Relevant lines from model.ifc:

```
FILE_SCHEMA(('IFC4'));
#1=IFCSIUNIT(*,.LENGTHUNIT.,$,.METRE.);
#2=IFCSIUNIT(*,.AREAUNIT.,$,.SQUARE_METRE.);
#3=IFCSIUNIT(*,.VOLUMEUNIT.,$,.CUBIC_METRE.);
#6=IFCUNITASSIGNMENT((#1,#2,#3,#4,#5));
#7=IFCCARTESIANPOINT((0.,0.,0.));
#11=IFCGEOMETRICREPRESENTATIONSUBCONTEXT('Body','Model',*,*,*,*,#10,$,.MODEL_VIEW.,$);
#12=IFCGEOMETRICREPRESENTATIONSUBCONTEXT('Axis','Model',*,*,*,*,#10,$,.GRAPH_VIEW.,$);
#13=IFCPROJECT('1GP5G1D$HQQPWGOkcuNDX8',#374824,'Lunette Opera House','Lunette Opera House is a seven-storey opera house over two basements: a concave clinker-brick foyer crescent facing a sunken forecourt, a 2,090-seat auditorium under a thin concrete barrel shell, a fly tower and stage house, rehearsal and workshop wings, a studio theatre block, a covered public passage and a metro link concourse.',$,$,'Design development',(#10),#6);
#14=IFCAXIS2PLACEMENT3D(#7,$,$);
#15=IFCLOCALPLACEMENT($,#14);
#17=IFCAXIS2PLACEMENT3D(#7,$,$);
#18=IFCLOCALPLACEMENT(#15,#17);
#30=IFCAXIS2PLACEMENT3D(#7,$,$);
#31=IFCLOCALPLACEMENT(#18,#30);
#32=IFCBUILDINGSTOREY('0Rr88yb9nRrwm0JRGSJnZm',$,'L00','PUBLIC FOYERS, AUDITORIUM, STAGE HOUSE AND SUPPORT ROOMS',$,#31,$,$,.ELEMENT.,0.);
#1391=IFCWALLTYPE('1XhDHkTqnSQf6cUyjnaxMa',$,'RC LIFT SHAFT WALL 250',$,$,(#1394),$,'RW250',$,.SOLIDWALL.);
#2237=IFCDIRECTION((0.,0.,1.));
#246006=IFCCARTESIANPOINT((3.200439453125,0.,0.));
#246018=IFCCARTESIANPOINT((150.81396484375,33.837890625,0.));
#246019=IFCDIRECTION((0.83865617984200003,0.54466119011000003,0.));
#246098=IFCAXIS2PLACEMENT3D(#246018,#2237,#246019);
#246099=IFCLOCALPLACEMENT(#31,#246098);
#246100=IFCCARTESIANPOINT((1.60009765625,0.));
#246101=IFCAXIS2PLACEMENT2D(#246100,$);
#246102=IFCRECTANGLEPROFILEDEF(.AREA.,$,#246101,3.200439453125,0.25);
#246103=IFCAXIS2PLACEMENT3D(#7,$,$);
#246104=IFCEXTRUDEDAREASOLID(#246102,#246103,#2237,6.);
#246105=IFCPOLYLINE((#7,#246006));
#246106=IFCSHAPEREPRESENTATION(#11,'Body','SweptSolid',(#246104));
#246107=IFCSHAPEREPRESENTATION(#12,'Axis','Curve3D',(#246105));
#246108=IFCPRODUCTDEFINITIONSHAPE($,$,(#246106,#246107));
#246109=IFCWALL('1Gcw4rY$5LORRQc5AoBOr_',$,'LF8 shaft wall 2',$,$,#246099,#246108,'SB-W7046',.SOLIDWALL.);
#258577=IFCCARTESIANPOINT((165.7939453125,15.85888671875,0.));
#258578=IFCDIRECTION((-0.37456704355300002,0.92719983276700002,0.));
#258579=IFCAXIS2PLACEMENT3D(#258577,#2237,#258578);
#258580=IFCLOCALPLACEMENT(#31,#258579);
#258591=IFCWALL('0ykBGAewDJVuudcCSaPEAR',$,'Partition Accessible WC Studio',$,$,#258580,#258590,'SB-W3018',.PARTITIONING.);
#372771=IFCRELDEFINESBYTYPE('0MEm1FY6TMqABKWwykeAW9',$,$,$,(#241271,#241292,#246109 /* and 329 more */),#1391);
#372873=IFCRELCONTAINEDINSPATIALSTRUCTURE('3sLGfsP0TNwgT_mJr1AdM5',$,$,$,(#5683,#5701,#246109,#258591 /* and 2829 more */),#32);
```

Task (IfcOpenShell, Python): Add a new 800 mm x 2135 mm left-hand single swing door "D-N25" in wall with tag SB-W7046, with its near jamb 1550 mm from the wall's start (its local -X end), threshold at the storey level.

```python
import numpy as np
import ifcopenshell
import ifcopenshell.api.feature
import ifcopenshell.api.geometry
import ifcopenshell.api.root
import ifcopenshell.api.spatial
import ifcopenshell.geom
import ifcopenshell.util.element
import ifcopenshell.util.placement
import ifcopenshell.util.representation
import ifcopenshell.util.shape
import ifcopenshell.util.unit

model = ifcopenshell.open("model.ifc")
unit_scale = ifcopenshell.util.unit.calculate_unit_scale(model)
settings = ifcopenshell.geom.settings()


def volume(element):
    """Net volume in cubic metres, openings subtracted."""
    shape = ifcopenshell.geom.create_shape(settings, element)
    return ifcopenshell.util.shape.get_volume(shape.geometry)


wall = model.by_id(246109)
storey = ifcopenshell.util.element.get_container(wall, ifc_class="IfcBuildingStorey")
context = ifcopenshell.util.representation.get_context(model, "Model", "Body", "MODEL_VIEW")
before = volume(wall)

width, height, from_end, sill = 0.8, 2.135, 1.55, 0.0  # metres

# The wall runs along its own X axis, and the end named is its -X end.
wall_shape = ifcopenshell.geom.create_shape(settings, wall)
x, y, z = ifcopenshell.util.shape.get_vertices(wall_shape.geometry).T
start = x.min() + from_end
face, thickness = float(y.min()), float(y.max() - y.min())
wall_matrix = ifcopenshell.util.placement.get_local_placement(wall.ObjectPlacement)
level = ifcopenshell.util.placement.get_local_placement(storey.ObjectPlacement)[2, 3]


def in_wall(x, y):
    """Placement at x, y metres in the wall's axes, at sill height."""
    matrix = wall_matrix.copy()
    matrix[:, 3] = wall_matrix @ np.array([x / unit_scale, y / unit_scale, 0.0, 1.0])
    matrix[2, 3] = level + sill / unit_scale
    return matrix


# Opening: a box that overshoots both wall faces by 50 mm.
opening = ifcopenshell.api.root.create_entity(model, ifc_class="IfcOpeningElement", predefined_type="OPENING")
box = ifcopenshell.api.geometry.add_wall_representation(
    model, context=context, length=width, height=height, thickness=thickness + 0.1
)
ifcopenshell.api.geometry.assign_representation(model, product=opening, representation=box)
ifcopenshell.api.geometry.edit_object_placement(model, product=opening, matrix=in_wall(start, face - 0.05), is_si=False)
ifcopenshell.api.feature.add_feature(model, feature=opening, element=wall)

door = ifcopenshell.api.root.create_entity(model, ifc_class="IfcDoor", name="D-N25", predefined_type="DOOR")
door.OverallWidth, door.OverallHeight = width / unit_scale, height / unit_scale
door.OperationType = "SINGLE_SWING_LEFT"
body = ifcopenshell.api.geometry.add_door_representation(
    model,
    context=context,
    overall_width=door.OverallWidth,
    overall_height=door.OverallHeight,
    operation_type="SINGLE_SWING_LEFT",
    lining_properties={"LiningDepth": thickness / unit_scale, "ThresholdDepth": thickness / unit_scale},
)
ifcopenshell.api.geometry.assign_representation(model, product=door, representation=body)
ifcopenshell.api.spatial.assign_container(model, products=[door], relating_structure=storey)
ifcopenshell.api.feature.add_filling(model, opening=opening, element=door)

# The lining spans the wall, so the door starts at the wall face.
ifcopenshell.api.geometry.edit_object_placement(model, product=door, matrix=in_wall(start, face), is_si=False)

after = volume(wall)

print(f"wall volume {before:.3f} -> {after:.3f} m3")

model.write("model_v2.ifc")
```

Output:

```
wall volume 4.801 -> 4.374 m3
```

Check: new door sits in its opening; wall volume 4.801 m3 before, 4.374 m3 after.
